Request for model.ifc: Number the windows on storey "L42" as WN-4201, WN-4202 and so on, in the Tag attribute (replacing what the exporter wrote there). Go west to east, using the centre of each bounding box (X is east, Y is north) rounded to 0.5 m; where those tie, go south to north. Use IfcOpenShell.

First a look at what the model holds.

```python
import ifcopenshell
import ifcopenshell.util.element
import ifcopenshell.util.placement

model = ifcopenshell.open("model.ifc")
print(model.schema)
storey = next(s for s in model.by_type("IfcBuildingStorey") if s.Name == "L42")
windows = [e for e in ifcopenshell.util.element.get_decomposition(storey) if e.is_a("IfcWindow")]
for e in sorted(windows, key=lambda e: e.id()):
    origin = ifcopenshell.util.placement.get_local_placement(e.ObjectPlacement)[:3, 3]
    print(e.id(), e.Tag, e.Name, origin.round(2) + 0.0, sep=" | ")
```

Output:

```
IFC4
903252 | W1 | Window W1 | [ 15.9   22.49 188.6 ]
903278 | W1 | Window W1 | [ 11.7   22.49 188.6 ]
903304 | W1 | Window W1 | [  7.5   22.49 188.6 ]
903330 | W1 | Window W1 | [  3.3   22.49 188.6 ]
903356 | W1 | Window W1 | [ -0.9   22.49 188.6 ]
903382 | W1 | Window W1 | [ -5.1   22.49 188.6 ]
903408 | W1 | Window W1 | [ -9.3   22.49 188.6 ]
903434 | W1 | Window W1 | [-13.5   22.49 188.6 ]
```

```python
import ifcopenshell
import ifcopenshell.geom
import ifcopenshell.util.element
import ifcopenshell.util.shape

model = ifcopenshell.open("model.ifc")
settings = ifcopenshell.geom.settings()
settings.set("use-world-coords", True)


def centre(element):
    shape = ifcopenshell.geom.create_shape(settings, element)
    return ifcopenshell.util.shape.get_bbox_centroid(shape.geometry)


storey = next(s for s in model.by_type("IfcBuildingStorey") if s.Name == "L42")
windows = [e for e in ifcopenshell.util.element.get_decomposition(storey) if e.is_a("IfcWindow")]

# Insertion points can sit at a corner or the storey origin, so sort by the geometry (in metres).
centres = {e: centre(e) for e in windows}
windows.sort(key=lambda e: (round(centres[e][0] / 0.5), centres[e][1]))

for i, e in enumerate(windows, start=1):
    number = f"WN-42{i:02d}"
    e.Tag = number
    print(e.id(), number)

model.write("model_edited.ifc")
```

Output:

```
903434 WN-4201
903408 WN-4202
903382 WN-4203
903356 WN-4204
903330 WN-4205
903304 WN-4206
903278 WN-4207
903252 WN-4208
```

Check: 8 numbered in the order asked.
